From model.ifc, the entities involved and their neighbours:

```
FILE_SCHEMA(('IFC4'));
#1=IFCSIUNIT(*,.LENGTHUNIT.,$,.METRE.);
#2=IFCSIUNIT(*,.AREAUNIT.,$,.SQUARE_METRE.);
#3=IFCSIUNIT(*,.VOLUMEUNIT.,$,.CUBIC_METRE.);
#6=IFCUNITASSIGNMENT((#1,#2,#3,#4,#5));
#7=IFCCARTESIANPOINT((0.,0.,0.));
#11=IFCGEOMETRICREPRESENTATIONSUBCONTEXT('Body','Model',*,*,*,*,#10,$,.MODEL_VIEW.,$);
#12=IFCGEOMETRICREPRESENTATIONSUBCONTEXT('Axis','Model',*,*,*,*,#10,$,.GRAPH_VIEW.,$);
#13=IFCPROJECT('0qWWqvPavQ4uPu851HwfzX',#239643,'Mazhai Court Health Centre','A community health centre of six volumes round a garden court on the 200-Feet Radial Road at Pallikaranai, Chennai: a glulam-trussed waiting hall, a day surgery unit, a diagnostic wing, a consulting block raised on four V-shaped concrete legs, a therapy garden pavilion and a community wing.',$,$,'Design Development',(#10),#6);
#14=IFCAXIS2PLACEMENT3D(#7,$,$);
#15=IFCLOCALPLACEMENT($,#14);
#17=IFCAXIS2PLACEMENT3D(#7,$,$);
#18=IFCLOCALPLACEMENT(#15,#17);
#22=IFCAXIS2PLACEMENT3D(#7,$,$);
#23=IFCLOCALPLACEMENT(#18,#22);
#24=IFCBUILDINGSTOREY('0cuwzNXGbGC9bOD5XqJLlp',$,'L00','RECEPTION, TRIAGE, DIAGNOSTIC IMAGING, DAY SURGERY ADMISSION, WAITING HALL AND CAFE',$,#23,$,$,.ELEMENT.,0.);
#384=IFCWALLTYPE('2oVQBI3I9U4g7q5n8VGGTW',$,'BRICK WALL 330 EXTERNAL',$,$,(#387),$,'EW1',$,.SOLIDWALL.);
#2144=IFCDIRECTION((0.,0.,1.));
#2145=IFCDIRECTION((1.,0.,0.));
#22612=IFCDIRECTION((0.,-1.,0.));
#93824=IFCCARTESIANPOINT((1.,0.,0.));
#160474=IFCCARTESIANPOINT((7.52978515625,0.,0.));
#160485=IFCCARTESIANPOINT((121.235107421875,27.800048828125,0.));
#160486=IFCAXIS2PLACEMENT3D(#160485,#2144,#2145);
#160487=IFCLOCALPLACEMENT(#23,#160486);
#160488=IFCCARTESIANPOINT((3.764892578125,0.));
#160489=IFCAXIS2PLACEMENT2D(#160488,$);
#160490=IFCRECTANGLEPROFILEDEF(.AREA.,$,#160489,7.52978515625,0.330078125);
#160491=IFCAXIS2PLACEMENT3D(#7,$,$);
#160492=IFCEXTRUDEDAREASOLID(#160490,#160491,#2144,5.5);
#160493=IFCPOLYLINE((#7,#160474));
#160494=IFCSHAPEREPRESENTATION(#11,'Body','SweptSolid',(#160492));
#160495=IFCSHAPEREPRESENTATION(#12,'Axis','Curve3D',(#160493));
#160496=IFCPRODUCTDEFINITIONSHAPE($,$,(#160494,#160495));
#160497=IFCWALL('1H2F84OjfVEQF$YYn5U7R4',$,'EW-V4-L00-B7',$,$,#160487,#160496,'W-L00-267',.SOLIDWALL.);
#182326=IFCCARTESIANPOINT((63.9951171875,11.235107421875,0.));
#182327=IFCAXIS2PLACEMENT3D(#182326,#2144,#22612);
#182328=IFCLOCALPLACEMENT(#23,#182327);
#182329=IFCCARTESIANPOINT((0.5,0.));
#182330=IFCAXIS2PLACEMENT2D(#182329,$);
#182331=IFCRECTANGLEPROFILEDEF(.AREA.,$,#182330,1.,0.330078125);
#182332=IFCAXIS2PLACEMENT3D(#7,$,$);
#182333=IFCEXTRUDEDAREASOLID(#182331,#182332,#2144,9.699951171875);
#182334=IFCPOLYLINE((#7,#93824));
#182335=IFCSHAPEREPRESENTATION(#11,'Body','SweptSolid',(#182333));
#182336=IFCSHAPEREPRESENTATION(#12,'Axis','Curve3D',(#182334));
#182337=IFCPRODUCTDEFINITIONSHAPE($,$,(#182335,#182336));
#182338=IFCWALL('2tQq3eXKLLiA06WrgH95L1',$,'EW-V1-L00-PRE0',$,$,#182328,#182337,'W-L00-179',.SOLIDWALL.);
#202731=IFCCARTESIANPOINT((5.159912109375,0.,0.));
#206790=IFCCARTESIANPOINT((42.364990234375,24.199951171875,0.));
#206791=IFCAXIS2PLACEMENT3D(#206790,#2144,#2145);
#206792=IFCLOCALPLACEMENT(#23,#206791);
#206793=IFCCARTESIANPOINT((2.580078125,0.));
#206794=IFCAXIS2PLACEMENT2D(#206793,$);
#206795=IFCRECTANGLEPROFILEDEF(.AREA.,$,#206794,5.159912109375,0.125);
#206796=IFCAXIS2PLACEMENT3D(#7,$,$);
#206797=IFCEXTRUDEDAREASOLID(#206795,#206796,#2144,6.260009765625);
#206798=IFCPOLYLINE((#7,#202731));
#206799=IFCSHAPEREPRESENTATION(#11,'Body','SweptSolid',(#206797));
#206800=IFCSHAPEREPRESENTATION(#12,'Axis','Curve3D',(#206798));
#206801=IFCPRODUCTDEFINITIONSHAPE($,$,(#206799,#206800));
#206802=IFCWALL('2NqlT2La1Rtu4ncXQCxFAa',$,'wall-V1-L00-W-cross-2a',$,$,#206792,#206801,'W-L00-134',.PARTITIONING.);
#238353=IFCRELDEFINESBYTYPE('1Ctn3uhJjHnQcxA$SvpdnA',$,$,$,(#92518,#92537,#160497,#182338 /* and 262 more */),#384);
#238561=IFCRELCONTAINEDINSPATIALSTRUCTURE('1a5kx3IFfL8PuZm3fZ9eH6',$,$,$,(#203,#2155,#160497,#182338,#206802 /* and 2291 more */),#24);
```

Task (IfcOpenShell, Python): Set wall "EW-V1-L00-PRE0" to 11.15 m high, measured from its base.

```python
import ifcopenshell
import ifcopenshell.geom
import ifcopenshell.util.representation
import ifcopenshell.util.shape
import ifcopenshell.util.unit

model = ifcopenshell.open("model.ifc")
unit_scale = ifcopenshell.util.unit.calculate_unit_scale(model)
settings = ifcopenshell.geom.settings()


def volume(element):
    """Net volume in cubic metres, openings subtracted."""
    shape = ifcopenshell.geom.create_shape(settings, element)
    return ifcopenshell.util.shape.get_volume(shape.geometry)


wall = model.by_guid("2tQq3eXKLLiA06WrgH95L1")
before = volume(wall)

body = ifcopenshell.util.representation.get_representation(wall, "Model", "Body")
solid = body.Items[0]
old_height = solid.Depth
solid.Depth = 11.15 / unit_scale
after = volume(wall)

print(f"height {old_height:g} -> {solid.Depth:g}, volume {before:.3f} -> {after:.3f} m3")

model.write("model_edited.ifc")
```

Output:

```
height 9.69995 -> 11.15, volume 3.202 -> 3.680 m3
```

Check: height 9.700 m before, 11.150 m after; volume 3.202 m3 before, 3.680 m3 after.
